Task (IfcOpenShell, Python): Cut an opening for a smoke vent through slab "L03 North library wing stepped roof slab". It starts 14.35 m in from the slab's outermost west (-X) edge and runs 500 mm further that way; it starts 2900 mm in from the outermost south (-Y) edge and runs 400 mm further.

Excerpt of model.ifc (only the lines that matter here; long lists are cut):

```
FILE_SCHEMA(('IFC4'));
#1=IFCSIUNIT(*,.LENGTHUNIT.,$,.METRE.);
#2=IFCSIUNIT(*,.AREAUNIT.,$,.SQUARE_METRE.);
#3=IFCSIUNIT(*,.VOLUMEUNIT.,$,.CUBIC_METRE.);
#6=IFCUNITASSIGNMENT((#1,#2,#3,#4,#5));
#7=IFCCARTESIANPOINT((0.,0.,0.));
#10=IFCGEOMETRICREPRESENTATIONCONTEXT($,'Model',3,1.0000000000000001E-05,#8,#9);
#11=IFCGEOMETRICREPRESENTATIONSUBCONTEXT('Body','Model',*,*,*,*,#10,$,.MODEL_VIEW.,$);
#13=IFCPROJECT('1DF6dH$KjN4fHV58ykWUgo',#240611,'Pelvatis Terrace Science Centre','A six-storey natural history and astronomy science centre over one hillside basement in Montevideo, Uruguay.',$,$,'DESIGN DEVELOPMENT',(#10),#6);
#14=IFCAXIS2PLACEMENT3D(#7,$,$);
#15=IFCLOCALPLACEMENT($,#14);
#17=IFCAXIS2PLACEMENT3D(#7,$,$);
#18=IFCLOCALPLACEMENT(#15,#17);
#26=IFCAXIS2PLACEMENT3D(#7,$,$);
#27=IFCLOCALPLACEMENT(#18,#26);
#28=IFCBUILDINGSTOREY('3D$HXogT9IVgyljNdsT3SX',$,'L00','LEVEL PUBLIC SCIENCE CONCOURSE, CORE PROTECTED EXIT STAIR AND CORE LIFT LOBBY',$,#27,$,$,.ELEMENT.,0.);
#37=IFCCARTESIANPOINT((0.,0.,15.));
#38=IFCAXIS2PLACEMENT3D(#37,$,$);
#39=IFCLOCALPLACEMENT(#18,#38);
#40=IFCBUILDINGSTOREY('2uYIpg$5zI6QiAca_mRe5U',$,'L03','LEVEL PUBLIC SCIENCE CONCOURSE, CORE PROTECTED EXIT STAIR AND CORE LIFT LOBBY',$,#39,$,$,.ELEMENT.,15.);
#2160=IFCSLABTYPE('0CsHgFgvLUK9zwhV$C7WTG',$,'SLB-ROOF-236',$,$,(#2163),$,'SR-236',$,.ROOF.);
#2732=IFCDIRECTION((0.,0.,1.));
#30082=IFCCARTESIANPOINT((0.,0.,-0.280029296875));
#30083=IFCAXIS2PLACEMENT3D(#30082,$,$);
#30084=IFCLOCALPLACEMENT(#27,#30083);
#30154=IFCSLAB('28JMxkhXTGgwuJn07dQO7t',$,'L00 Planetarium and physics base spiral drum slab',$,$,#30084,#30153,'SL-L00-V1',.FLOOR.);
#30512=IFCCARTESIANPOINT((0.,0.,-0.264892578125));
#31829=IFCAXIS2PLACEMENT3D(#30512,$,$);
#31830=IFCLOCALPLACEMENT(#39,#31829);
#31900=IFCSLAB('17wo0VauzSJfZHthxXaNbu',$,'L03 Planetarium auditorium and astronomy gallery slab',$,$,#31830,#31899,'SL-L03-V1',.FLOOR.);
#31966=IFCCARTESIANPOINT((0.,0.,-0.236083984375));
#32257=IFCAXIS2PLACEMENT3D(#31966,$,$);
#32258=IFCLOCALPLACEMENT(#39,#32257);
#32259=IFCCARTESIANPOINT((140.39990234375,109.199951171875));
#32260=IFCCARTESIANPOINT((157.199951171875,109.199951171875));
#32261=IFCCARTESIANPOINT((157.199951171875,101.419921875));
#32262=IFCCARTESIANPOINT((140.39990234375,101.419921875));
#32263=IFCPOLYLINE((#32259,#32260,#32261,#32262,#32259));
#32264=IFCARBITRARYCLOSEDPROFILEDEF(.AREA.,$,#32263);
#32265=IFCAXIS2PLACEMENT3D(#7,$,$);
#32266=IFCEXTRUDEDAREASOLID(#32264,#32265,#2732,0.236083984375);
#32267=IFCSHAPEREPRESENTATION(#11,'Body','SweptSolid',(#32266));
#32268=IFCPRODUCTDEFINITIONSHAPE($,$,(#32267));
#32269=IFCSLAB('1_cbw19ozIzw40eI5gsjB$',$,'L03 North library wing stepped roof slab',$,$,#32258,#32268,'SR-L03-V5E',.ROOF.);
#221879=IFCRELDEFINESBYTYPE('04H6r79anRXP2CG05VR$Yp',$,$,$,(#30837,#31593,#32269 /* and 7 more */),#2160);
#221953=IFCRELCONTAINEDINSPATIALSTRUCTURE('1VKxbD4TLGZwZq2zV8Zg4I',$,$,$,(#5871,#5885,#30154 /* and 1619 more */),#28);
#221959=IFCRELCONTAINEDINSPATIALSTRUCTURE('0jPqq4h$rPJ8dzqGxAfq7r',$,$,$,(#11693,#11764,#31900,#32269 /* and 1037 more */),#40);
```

```python
import numpy as np
import ifcopenshell
import ifcopenshell.api.feature
import ifcopenshell.api.geometry
import ifcopenshell.api.root
import ifcopenshell.geom
import ifcopenshell.util.placement
import ifcopenshell.util.representation
import ifcopenshell.util.shape
import ifcopenshell.util.unit

model = ifcopenshell.open("model.ifc")
unit_scale = ifcopenshell.util.unit.calculate_unit_scale(model)
settings = ifcopenshell.geom.settings()


def volume(element):
    """Net volume in cubic metres, openings subtracted."""
    shape = ifcopenshell.geom.create_shape(settings, element)
    return ifcopenshell.util.shape.get_volume(shape.geometry)


slab = model.by_guid("1_cbw19ozIzw40eI5gsjB$")
before = volume(slab)

# Extent in the slab's own axes, in metres. The edges named are its -X and -Y sides.
slab_shape = ifcopenshell.geom.create_shape(settings, slab)
vertices = ifcopenshell.util.shape.get_vertices(slab_shape.geometry)
x_min, y_min, bottom = vertices.min(axis=0)
top = vertices[:, 2].max()

opening = ifcopenshell.api.root.create_entity(model, ifc_class="IfcOpeningElement", name="Smoke vent opening", predefined_type="OPENING")
context = ifcopenshell.util.representation.get_context(model, "Model", "Body", "MODEL_VIEW")
width, depth = 0.5, 0.4
outline = [(0.0, 0.0), (width, 0.0), (width, depth), (0.0, depth), (0.0, 0.0)]
# Overshoot both faces by 50 mm so the cut is clean.
shape = ifcopenshell.api.geometry.add_slab_representation(
    model, context=context, depth=top - bottom + 0.1, polyline=outline
)
ifcopenshell.api.geometry.assign_representation(model, product=opening, representation=shape)

matrix = ifcopenshell.util.placement.get_local_placement(slab.ObjectPlacement)
matrix[:, 3] = matrix @ np.append(np.array([x_min + 14.35, y_min + 2.9, bottom - 0.05]) / unit_scale, 1.0)
ifcopenshell.api.geometry.edit_object_placement(model, product=opening, matrix=matrix, is_si=False)
ifcopenshell.api.feature.add_feature(model, feature=opening, element=slab)

after = volume(slab)

print(f"slab volume {before:.3f} -> {after:.3f} m3")

model.write("model_v2.ifc")
```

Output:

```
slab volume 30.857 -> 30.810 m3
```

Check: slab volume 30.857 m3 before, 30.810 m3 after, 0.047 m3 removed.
